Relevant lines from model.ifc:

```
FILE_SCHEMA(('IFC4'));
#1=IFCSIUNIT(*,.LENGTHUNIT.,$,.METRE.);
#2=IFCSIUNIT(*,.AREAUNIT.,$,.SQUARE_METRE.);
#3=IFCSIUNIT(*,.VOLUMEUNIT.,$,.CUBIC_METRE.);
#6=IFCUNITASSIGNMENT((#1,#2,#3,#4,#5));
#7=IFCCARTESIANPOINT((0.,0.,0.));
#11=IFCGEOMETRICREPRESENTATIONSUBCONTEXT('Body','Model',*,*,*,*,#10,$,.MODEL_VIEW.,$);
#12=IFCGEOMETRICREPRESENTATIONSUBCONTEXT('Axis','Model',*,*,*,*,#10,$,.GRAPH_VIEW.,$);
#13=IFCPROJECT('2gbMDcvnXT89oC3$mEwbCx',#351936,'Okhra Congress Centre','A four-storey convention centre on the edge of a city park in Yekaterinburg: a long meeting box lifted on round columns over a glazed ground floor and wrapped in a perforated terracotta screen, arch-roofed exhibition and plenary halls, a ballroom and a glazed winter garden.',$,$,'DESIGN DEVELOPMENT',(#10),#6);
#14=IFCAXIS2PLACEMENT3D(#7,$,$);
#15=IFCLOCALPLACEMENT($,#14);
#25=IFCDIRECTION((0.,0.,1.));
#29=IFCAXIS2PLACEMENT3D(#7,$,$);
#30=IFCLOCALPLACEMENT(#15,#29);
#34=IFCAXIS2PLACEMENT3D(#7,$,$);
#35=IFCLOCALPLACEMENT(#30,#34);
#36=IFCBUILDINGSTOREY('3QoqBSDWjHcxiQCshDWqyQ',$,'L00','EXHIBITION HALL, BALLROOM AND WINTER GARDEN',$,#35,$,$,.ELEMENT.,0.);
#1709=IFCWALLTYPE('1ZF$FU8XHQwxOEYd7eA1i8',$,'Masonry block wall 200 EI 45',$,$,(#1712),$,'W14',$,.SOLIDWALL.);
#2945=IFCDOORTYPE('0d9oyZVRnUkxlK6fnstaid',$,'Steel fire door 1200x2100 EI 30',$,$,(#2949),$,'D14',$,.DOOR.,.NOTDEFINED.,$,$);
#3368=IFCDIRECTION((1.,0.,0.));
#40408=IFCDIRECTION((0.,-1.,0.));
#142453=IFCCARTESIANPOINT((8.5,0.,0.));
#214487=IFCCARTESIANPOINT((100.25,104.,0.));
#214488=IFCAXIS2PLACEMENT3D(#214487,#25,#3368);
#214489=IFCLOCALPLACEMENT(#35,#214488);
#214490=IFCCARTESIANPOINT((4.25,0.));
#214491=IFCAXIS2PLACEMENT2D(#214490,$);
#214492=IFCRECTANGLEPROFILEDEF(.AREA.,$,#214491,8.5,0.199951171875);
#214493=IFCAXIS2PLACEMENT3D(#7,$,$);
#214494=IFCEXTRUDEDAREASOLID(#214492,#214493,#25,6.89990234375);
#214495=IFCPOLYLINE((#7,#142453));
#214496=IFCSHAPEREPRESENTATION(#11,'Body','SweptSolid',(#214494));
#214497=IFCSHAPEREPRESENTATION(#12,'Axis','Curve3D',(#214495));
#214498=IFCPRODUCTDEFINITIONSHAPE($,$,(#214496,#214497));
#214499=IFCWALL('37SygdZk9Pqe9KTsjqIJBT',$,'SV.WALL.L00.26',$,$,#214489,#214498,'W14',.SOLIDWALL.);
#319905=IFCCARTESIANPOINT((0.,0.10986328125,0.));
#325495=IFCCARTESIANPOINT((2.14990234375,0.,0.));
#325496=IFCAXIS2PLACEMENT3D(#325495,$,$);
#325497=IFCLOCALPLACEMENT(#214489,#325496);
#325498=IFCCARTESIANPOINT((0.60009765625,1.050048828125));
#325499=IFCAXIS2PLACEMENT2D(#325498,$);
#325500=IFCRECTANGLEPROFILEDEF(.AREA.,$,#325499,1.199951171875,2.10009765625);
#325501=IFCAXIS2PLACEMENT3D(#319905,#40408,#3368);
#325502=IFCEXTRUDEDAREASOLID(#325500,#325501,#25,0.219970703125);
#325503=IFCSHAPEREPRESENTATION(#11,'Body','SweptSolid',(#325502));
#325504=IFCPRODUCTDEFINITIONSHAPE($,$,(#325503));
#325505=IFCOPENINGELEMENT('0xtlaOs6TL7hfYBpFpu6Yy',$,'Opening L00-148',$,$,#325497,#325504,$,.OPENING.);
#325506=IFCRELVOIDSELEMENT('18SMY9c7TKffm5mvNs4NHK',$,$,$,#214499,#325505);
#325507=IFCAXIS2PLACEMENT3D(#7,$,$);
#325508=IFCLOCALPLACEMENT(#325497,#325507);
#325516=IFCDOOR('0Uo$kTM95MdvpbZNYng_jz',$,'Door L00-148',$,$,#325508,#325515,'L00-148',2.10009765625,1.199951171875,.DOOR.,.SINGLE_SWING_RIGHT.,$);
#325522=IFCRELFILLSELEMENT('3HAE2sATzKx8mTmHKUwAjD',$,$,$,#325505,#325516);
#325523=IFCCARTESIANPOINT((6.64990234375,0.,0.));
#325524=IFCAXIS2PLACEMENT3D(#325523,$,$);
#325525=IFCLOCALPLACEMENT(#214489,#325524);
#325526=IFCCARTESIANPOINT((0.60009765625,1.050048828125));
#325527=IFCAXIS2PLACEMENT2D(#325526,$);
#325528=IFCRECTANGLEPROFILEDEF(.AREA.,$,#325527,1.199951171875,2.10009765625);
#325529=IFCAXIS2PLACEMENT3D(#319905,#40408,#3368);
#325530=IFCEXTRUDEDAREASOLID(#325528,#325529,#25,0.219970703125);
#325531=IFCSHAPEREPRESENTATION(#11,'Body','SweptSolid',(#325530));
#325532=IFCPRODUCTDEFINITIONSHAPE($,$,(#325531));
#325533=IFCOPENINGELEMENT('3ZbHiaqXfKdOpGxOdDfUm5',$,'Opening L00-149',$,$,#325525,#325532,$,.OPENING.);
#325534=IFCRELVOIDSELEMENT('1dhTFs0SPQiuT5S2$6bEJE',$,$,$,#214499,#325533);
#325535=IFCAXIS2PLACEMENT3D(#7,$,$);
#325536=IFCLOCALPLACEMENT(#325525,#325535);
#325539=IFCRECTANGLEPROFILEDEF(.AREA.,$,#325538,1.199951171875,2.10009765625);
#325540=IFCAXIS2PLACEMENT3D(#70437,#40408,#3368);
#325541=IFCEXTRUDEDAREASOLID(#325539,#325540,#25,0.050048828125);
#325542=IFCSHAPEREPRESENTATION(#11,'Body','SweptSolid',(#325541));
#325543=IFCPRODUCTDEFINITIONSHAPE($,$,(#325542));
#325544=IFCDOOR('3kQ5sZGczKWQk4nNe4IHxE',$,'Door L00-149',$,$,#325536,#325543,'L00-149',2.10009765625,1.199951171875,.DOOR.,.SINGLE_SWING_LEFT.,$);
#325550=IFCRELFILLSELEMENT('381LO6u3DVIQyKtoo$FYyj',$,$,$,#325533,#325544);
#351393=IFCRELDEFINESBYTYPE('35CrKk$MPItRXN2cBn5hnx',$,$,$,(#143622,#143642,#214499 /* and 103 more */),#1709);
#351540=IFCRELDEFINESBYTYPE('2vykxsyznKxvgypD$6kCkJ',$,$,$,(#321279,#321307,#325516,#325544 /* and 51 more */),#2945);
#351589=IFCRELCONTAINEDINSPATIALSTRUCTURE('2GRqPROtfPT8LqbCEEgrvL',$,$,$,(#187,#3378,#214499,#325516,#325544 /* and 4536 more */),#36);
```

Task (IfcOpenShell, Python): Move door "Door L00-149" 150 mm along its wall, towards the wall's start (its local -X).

```python
import ifcopenshell
import ifcopenshell.api.geometry
import ifcopenshell.util.placement
import ifcopenshell.util.unit

model = ifcopenshell.open("model.ifc")
unit_scale = ifcopenshell.util.unit.calculate_unit_scale(model)

door = model.by_id(325544)
opening = door.FillsVoids[0].RelatingOpeningElement
wall = opening.VoidsElements[0].RelatingBuildingElement

wall_matrix = ifcopenshell.util.placement.get_local_placement(wall.ObjectPlacement)
shift = wall_matrix[:3, 0] * -0.15 / unit_scale
before = ifcopenshell.util.placement.get_local_placement(door.ObjectPlacement)[:3, 3].copy()

# The door is placed relative to its opening, so it follows when the opening moves.
matrix = ifcopenshell.util.placement.get_local_placement(opening.ObjectPlacement)
matrix[:3, 3] += shift
ifcopenshell.api.geometry.edit_object_placement(
    model, product=opening, matrix=matrix, is_si=False, should_transform_children=True
)

after = ifcopenshell.util.placement.get_local_placement(door.ObjectPlacement)[:3, 3]
print("door moved by", (after - before).round(3) + 0.0)

model.write("model_updated.ifc")
```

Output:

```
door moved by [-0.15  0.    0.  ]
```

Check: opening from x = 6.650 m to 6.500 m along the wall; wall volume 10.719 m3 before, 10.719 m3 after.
